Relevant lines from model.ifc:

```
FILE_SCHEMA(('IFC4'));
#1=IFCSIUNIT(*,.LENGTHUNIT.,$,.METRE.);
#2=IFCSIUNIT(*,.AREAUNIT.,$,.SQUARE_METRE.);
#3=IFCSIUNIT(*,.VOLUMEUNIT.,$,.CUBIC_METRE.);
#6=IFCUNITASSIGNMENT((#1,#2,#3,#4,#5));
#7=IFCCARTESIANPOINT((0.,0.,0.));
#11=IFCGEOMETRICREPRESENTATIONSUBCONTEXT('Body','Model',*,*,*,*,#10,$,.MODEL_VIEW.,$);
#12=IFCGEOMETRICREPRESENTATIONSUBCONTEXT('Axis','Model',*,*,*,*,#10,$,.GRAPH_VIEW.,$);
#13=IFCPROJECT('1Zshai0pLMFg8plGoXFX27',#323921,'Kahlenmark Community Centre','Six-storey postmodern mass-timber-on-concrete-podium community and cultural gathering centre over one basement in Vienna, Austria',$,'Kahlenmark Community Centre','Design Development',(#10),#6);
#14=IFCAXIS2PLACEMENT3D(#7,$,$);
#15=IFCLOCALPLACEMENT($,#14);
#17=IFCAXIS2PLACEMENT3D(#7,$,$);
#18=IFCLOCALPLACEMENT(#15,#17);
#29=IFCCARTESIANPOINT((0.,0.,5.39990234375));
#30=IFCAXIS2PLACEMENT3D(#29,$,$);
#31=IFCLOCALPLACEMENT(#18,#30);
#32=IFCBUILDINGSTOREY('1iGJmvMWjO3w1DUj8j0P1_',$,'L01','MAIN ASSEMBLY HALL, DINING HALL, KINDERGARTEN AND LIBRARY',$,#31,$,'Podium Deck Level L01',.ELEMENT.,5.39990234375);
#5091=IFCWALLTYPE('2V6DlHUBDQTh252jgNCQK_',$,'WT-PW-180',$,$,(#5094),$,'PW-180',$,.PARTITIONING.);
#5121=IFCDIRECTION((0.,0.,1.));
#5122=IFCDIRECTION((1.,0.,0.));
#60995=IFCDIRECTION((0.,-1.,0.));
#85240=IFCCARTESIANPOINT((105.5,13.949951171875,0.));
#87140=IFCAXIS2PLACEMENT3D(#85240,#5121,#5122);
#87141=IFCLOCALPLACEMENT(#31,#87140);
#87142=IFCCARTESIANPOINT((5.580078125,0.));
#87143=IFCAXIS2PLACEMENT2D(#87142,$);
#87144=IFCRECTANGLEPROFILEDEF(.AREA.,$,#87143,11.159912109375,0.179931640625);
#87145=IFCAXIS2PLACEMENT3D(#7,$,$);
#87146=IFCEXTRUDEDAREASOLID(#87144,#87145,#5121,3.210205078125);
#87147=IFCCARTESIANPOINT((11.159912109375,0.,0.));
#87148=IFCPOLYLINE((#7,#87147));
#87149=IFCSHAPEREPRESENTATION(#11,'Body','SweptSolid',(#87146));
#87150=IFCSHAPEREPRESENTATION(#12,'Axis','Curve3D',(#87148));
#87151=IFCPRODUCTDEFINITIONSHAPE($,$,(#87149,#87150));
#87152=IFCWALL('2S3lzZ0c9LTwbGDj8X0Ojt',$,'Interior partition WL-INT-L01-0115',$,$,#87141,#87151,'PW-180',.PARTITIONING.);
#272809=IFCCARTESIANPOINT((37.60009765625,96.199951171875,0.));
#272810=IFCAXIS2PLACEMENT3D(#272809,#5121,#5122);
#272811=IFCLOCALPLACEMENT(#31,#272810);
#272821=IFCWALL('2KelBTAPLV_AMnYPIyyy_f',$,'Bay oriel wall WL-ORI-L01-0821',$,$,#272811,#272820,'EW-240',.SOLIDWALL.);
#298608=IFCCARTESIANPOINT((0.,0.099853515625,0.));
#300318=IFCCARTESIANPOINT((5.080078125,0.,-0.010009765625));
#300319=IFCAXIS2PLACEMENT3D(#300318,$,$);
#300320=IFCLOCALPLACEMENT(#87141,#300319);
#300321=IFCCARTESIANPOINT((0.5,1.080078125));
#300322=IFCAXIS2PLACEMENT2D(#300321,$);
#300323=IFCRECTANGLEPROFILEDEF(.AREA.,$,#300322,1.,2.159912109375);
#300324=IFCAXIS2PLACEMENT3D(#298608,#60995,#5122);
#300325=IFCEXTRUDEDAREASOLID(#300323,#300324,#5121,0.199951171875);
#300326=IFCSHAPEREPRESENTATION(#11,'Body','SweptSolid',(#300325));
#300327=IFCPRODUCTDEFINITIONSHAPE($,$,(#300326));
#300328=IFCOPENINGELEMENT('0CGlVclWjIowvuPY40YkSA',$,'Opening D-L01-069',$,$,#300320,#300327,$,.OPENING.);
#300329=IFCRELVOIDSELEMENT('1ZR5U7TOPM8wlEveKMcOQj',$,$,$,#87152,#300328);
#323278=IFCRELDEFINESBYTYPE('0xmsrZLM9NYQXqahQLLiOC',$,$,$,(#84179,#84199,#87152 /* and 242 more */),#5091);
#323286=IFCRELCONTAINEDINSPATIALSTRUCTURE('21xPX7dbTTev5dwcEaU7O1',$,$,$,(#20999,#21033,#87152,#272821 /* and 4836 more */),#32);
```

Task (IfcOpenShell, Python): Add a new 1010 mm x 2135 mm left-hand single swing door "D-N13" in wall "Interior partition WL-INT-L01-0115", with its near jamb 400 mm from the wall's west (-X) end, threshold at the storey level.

```python
import numpy as np
import ifcopenshell
import ifcopenshell.api.feature
import ifcopenshell.api.geometry
import ifcopenshell.api.root
import ifcopenshell.api.spatial
import ifcopenshell.geom
import ifcopenshell.util.element
import ifcopenshell.util.placement
import ifcopenshell.util.representation
import ifcopenshell.util.shape
import ifcopenshell.util.unit

model = ifcopenshell.open("model.ifc")
unit_scale = ifcopenshell.util.unit.calculate_unit_scale(model)
settings = ifcopenshell.geom.settings()


def volume(element):
    """Net volume in cubic metres, openings subtracted."""
    shape = ifcopenshell.geom.create_shape(settings, element)
    return ifcopenshell.util.shape.get_volume(shape.geometry)


wall = model.by_guid("2S3lzZ0c9LTwbGDj8X0Ojt")
storey = ifcopenshell.util.element.get_container(wall, ifc_class="IfcBuildingStorey")
context = ifcopenshell.util.representation.get_context(model, "Model", "Body", "MODEL_VIEW")
before = volume(wall)

width, height, from_end, sill = 1.01, 2.135, 0.4, 0.0  # metres

# The wall runs along its own X axis, and the end named is its -X end.
wall_shape = ifcopenshell.geom.create_shape(settings, wall)
x, y, z = ifcopenshell.util.shape.get_vertices(wall_shape.geometry).T
start = x.min() + from_end
face, thickness = float(y.min()), float(y.max() - y.min())
wall_matrix = ifcopenshell.util.placement.get_local_placement(wall.ObjectPlacement)
level = ifcopenshell.util.placement.get_local_placement(storey.ObjectPlacement)[2, 3]


def in_wall(x, y):
    """Placement at x, y metres in the wall's axes, at sill height."""
    matrix = wall_matrix.copy()
    matrix[:, 3] = wall_matrix @ np.array([x / unit_scale, y / unit_scale, 0.0, 1.0])
    matrix[2, 3] = level + sill / unit_scale
    return matrix


# Opening: a box that overshoots both wall faces by 50 mm.
opening = ifcopenshell.api.root.create_entity(model, ifc_class="IfcOpeningElement", predefined_type="OPENING")
box = ifcopenshell.api.geometry.add_wall_representation(
    model, context=context, length=width, height=height, thickness=thickness + 0.1
)
ifcopenshell.api.geometry.assign_representation(model, product=opening, representation=box)
ifcopenshell.api.geometry.edit_object_placement(model, product=opening, matrix=in_wall(start, face - 0.05), is_si=False)
ifcopenshell.api.feature.add_feature(model, feature=opening, element=wall)

door = ifcopenshell.api.root.create_entity(model, ifc_class="IfcDoor", name="D-N13", predefined_type="DOOR")
door.OverallWidth, door.OverallHeight = width / unit_scale, height / unit_scale
door.OperationType = "SINGLE_SWING_LEFT"
body = ifcopenshell.api.geometry.add_door_representation(
    model,
    context=context,
    overall_width=door.OverallWidth,
    overall_height=door.OverallHeight,
    operation_type="SINGLE_SWING_LEFT",
    lining_properties={"LiningDepth": thickness / unit_scale, "ThresholdDepth": thickness / unit_scale},
)
ifcopenshell.api.geometry.assign_representation(model, product=door, representation=body)
ifcopenshell.api.spatial.assign_container(model, products=[door], relating_structure=storey)
ifcopenshell.api.feature.add_filling(model, opening=opening, element=door)

# The lining spans the wall, so the door starts at the wall face.
ifcopenshell.api.geometry.edit_object_placement(model, product=door, matrix=in_wall(start, face), is_si=False)

after = volume(wall)

print(f"wall volume {before:.3f} -> {after:.3f} m3")

model.write("model_updated.ifc")
```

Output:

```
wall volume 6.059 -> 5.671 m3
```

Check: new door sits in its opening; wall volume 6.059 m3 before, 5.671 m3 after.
